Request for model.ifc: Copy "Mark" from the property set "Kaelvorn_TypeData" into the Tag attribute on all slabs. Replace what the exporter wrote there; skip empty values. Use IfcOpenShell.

First a look at what the model holds.

```python
import ifcopenshell
import ifcopenshell.util.element

model = ifcopenshell.open("model.ifc")
print(model.schema)
slabs = model.by_type("IfcSlab")
print(len(slabs), "slabs")
for e in slabs[:8]:
    source = ifcopenshell.util.element.get_pset(e, "Kaelvorn_TypeData", "Mark")
    target = e.Tag
    print(e.id(), repr(source), repr(target), sep=" | ")
```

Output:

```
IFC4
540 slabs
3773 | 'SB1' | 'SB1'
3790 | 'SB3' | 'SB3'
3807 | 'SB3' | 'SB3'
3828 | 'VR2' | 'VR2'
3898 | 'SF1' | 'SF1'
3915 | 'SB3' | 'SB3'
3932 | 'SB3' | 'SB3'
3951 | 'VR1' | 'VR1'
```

```python
import ifcopenshell
import ifcopenshell.util.element

model = ifcopenshell.open("model.ifc")

count = 0
for e in model.by_type("IfcSlab"):
    value = ifcopenshell.util.element.get_pset(e, "Kaelvorn_TypeData", "Mark")
    current = e.Tag
    if not value or not value.strip() or current == value:
        continue
    e.Tag = value
    count += 1

print(count, "slabs updated")

model.write("model_edited.ifc")
```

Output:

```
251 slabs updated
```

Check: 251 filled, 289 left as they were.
